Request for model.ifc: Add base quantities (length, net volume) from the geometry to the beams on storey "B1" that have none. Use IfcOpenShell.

First a look at what the model holds.

```python
import ifcopenshell
import ifcopenshell.util.element
import ifcopenshell.util.unit

model = ifcopenshell.open("model.ifc")
print(model.schema)
for unit_type in ("LENGTHUNIT", "AREAUNIT", "VOLUMEUNIT"):
    print(unit_type, ifcopenshell.util.unit.calculate_unit_scale(model, unit_type))
storey = next(s for s in model.by_type("IfcBuildingStorey") if s.Name == "B1")
beams = [e for e in ifcopenshell.util.element.get_decomposition(storey) if e.is_a("IfcBeam")]
for e in sorted(beams, key=lambda e: e.id()):
    print(e.id(), e.is_a(), e.Name, list(ifcopenshell.util.element.get_psets(e, qtos_only=True)), sep=" | ")
```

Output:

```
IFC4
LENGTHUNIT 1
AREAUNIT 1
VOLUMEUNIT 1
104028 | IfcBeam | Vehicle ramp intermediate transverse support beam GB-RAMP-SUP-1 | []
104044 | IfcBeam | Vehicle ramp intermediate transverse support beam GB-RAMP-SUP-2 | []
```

```python
import ifcopenshell
import ifcopenshell.api.pset
import ifcopenshell.geom
import ifcopenshell.util.element
import ifcopenshell.util.shape
import ifcopenshell.util.unit

model = ifcopenshell.open("model.ifc")
unit_scale = ifcopenshell.util.unit.calculate_unit_scale(model)
volume_scale = ifcopenshell.util.unit.calculate_unit_scale(model, "VOLUMEUNIT")
settings = ifcopenshell.geom.settings()

storey = next(s for s in model.by_type("IfcBuildingStorey") if s.Name == "B1")
beams = [e for e in ifcopenshell.util.element.get_decomposition(storey) if e.is_a("IfcBeam")]

for e in sorted(beams, key=lambda e: e.id()):
    if ifcopenshell.util.element.get_psets(e, qtos_only=True, should_inherit=False):
        continue
    # Geometry comes back in metres, in the element's own axes.
    shape = ifcopenshell.geom.create_shape(settings, e)
    values = {
        "Length": ifcopenshell.util.shape.get_max_xyz(shape.geometry) / unit_scale,
        "NetVolume": ifcopenshell.util.shape.get_volume(shape.geometry) / volume_scale,
    }
    qto = ifcopenshell.api.pset.add_qto(model, product=e, name="Qto_BeamBaseQuantities")
    ifcopenshell.api.pset.edit_qto(model, qto=qto, properties=values)
    print(e.id(), {k: round(v, 3) for k, v in values.items()})

model.write("model_rev.ifc")
```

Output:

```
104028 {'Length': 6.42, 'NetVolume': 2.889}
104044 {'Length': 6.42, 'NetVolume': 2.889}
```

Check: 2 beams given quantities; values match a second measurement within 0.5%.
